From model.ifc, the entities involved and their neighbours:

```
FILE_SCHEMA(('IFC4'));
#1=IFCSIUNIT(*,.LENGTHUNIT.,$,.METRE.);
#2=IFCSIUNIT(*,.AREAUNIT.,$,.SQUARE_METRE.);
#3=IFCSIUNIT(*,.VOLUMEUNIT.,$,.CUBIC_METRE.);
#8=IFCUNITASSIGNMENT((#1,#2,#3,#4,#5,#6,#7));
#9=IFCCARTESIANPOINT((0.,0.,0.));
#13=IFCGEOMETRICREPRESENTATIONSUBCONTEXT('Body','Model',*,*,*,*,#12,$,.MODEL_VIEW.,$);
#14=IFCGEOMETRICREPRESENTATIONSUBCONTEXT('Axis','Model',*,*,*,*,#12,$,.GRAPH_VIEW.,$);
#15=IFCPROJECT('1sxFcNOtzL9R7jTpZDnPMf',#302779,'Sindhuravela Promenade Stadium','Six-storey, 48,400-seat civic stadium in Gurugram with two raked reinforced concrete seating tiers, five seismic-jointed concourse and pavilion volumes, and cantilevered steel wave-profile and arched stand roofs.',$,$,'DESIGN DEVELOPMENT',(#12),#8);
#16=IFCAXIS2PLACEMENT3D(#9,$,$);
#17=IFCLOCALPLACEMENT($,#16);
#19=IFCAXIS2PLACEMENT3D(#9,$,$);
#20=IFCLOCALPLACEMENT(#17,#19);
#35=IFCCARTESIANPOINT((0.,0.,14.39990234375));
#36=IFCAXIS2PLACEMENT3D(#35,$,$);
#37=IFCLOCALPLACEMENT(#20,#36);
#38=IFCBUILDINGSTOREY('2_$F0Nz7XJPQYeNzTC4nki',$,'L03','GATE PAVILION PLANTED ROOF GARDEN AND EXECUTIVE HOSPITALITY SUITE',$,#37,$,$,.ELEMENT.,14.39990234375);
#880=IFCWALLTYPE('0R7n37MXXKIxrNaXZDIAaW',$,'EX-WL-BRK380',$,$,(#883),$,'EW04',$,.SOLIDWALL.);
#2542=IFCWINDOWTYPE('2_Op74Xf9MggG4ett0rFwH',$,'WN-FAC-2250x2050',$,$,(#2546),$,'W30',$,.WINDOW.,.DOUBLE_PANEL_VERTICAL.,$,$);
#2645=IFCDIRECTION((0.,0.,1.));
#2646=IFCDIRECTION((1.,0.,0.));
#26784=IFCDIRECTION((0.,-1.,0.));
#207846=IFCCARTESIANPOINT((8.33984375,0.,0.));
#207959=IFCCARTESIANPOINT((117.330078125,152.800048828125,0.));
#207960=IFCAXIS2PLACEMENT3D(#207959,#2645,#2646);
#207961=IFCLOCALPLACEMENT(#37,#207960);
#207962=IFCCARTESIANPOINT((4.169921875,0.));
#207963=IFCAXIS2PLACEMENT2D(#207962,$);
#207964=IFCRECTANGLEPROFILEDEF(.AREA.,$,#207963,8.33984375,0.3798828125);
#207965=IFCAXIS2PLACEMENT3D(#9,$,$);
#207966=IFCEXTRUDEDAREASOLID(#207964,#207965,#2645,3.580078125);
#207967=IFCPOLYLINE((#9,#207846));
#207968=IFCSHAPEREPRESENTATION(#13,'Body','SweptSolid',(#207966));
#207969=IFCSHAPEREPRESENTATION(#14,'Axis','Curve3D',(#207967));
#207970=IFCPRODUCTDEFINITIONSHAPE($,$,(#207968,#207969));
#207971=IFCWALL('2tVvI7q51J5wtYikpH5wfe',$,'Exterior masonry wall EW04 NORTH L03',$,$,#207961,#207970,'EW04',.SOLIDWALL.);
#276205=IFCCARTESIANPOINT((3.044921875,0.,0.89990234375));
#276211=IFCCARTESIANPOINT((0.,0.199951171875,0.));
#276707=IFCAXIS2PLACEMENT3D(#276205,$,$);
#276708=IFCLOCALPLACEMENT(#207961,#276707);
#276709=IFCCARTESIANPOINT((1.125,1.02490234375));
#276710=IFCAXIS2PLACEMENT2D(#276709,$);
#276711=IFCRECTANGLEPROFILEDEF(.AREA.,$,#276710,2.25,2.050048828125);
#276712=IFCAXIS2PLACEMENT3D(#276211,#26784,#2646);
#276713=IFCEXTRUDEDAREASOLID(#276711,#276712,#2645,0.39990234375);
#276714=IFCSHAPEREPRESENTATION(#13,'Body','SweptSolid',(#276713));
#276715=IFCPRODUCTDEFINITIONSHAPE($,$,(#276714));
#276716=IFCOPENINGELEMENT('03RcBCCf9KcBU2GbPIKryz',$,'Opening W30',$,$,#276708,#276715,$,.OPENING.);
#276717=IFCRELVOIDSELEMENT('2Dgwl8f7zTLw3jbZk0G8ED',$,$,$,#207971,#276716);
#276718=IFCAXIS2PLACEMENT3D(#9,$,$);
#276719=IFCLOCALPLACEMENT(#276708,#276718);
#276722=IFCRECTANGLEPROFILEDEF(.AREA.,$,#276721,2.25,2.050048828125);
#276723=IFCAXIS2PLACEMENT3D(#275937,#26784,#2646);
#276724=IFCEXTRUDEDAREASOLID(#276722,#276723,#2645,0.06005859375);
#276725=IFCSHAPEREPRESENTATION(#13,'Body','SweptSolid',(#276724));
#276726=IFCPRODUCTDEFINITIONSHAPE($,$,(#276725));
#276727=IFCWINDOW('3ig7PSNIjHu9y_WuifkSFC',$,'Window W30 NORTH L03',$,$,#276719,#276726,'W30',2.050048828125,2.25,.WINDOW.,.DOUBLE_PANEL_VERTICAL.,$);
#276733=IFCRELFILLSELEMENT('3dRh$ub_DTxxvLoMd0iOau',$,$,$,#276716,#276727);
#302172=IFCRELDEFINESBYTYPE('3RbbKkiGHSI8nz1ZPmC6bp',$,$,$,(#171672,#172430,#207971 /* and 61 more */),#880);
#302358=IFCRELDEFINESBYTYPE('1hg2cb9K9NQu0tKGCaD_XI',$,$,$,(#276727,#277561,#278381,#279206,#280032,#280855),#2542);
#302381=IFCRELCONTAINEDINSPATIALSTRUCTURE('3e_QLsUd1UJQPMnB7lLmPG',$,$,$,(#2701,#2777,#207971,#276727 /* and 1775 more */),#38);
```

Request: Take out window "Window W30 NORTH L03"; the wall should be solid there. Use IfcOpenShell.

```python
import ifcopenshell
import ifcopenshell.api.feature
import ifcopenshell.api.root
import ifcopenshell.geom
import ifcopenshell.util.shape

model = ifcopenshell.open("model.ifc")
settings = ifcopenshell.geom.settings()


def volume(element):
    """Net volume in cubic metres, openings subtracted."""
    shape = ifcopenshell.geom.create_shape(settings, element)
    return ifcopenshell.util.shape.get_volume(shape.geometry)


window = model.by_guid("3ig7PSNIjHu9y_WuifkSFC")
opening = window.FillsVoids[0].RelatingOpeningElement
wall = opening.VoidsElements[0].RelatingBuildingElement
before = volume(wall)

ifcopenshell.api.root.remove_product(model, product=window)
ifcopenshell.api.feature.remove_feature(model, feature=opening)

after = volume(wall)

print(f"wall volume {before:.3f} -> {after:.3f} m3")

model.write("model-out.ifc")
```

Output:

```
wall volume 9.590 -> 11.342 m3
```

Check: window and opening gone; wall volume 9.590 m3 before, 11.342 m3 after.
